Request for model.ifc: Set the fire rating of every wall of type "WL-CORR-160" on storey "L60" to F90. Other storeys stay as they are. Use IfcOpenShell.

First a look at what the model holds.

```python
import ifcopenshell
import ifcopenshell.util.element

model = ifcopenshell.open("model.ifc")
print(model.schema)
storey = next(s for s in model.by_type("IfcBuildingStorey") if s.Name == "L60")
walls = [e for e in ifcopenshell.util.element.get_decomposition(storey) if e.is_a("IfcWall")]
seen = {}
for e in walls:
    element_type = ifcopenshell.util.element.get_type(e)
    key = (element_type.Name if element_type != e and element_type else None, ifcopenshell.util.element.get_pset(e, "Pset_WallCommon", "FireRating"))
    seen[key] = seen.get(key, 0) + 1
for (name, value), count in sorted(seen.items(), key=str):
    print(count, "x", name, "|", value)
```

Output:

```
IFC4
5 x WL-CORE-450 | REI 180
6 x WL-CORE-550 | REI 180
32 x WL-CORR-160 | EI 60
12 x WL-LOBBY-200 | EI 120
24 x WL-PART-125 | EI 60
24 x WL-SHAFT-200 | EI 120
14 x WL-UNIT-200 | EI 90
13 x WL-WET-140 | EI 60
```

```python
import ifcopenshell
import ifcopenshell.api.pset
import ifcopenshell.util.element

model = ifcopenshell.open("model.ifc")

storey = next(s for s in model.by_type("IfcBuildingStorey") if s.Name == "L60")
walls = [e for e in ifcopenshell.util.element.get_decomposition(storey) if e.is_a("IfcWall")]

count = 0
for e in walls:
    element_type = ifcopenshell.util.element.get_type(e)
    if element_type in (None, e) or element_type.Name != "WL-CORR-160":
        continue
    # add_pset returns the element's existing set when there is one.
    pset = ifcopenshell.api.pset.add_pset(model, product=e, name="Pset_WallCommon")
    ifcopenshell.api.pset.edit_pset(model, pset=pset, properties={"FireRating": "F90"})
    count += 1

print(count, "walls updated")

model.write("model_v2.ifc")
```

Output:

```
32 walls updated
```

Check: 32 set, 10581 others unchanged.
